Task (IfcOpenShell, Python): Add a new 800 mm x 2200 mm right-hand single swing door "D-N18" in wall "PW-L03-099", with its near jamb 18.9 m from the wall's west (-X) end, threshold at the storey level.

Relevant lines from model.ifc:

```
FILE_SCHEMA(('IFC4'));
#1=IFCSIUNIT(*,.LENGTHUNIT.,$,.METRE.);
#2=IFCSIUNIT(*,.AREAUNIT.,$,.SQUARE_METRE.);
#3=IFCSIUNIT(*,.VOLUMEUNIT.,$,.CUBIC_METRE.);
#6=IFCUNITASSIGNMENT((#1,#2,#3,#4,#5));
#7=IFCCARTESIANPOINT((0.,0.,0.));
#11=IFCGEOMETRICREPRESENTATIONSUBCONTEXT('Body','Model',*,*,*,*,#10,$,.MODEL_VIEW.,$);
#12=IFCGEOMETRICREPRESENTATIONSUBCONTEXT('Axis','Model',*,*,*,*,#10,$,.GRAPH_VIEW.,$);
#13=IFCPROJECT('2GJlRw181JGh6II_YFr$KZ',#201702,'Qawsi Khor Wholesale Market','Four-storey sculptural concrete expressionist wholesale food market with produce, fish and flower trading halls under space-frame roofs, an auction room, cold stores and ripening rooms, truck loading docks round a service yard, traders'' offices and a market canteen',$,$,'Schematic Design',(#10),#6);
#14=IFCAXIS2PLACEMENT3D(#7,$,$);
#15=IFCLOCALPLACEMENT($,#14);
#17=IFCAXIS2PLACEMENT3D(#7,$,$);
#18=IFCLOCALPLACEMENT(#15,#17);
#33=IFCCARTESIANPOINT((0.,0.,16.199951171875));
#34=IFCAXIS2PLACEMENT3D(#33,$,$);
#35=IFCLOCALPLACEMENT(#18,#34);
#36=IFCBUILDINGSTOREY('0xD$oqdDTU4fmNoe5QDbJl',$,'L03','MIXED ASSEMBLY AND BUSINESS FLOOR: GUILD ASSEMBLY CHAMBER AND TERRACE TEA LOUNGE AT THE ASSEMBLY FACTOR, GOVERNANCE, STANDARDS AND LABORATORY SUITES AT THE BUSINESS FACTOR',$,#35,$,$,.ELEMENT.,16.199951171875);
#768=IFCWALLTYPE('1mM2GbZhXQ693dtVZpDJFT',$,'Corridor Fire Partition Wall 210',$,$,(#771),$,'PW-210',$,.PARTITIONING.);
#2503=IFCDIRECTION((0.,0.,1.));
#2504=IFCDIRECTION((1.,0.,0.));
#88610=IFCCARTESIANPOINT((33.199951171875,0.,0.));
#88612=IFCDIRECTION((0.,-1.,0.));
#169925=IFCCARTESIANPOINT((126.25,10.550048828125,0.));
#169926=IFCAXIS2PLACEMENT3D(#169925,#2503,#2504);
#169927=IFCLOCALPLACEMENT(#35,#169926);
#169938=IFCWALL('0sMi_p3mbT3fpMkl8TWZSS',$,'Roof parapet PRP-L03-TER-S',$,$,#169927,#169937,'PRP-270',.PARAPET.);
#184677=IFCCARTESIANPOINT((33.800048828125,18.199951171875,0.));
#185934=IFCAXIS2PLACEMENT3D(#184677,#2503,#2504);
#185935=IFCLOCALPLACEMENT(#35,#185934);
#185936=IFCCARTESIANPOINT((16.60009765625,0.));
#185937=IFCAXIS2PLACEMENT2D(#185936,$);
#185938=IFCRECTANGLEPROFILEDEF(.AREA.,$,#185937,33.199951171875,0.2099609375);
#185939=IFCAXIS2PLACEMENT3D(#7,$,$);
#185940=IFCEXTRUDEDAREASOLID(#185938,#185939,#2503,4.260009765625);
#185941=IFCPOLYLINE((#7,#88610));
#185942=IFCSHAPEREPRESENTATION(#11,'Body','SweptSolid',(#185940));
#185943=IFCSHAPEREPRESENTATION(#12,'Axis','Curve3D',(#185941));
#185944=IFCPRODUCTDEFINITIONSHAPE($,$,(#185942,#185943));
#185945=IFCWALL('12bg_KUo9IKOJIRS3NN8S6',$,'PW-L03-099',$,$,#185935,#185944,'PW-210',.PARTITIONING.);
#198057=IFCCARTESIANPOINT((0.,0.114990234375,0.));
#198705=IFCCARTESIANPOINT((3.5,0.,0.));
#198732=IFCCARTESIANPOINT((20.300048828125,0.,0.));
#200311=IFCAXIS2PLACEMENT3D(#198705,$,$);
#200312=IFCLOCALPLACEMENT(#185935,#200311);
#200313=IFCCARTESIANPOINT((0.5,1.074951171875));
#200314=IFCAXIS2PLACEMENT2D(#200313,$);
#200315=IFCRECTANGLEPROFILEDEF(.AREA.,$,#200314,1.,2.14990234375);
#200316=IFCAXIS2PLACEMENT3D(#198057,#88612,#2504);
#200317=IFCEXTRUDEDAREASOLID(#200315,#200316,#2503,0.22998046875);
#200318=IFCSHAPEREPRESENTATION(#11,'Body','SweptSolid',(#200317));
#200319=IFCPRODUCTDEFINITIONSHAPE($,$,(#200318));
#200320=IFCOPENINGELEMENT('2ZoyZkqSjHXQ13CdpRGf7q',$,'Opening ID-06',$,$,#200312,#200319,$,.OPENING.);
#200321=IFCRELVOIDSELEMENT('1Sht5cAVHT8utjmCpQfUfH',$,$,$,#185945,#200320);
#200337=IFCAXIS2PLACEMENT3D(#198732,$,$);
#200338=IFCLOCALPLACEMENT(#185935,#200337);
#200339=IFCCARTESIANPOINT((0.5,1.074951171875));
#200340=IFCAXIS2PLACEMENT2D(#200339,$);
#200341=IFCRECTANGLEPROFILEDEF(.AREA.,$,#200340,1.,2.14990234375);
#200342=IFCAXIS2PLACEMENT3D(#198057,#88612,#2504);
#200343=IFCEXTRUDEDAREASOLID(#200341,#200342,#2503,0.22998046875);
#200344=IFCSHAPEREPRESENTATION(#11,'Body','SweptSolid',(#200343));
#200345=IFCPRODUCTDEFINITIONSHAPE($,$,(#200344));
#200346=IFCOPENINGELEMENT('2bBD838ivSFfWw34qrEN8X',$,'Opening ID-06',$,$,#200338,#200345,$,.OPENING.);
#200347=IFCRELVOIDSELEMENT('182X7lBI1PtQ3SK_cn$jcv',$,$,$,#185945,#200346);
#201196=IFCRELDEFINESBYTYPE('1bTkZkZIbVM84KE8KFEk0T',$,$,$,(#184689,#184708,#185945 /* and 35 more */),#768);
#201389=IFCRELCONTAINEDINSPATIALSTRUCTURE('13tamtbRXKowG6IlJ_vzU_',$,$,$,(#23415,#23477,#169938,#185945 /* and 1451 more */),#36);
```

```python
import numpy as np
import ifcopenshell
import ifcopenshell.api.feature
import ifcopenshell.api.geometry
import ifcopenshell.api.root
import ifcopenshell.api.spatial
import ifcopenshell.geom
import ifcopenshell.util.element
import ifcopenshell.util.placement
import ifcopenshell.util.representation
import ifcopenshell.util.shape
import ifcopenshell.util.unit

model = ifcopenshell.open("model.ifc")
unit_scale = ifcopenshell.util.unit.calculate_unit_scale(model)
settings = ifcopenshell.geom.settings()


def volume(element):
    """Net volume in cubic metres, openings subtracted."""
    shape = ifcopenshell.geom.create_shape(settings, element)
    return ifcopenshell.util.shape.get_volume(shape.geometry)


wall = model.by_guid("12bg_KUo9IKOJIRS3NN8S6")
storey = ifcopenshell.util.element.get_container(wall, ifc_class="IfcBuildingStorey")
context = ifcopenshell.util.representation.get_context(model, "Model", "Body", "MODEL_VIEW")
before = volume(wall)

width, height, from_end, sill = 0.8, 2.2, 18.9, 0.0  # metres

# The wall runs along its own X axis, and the end named is its -X end.
wall_shape = ifcopenshell.geom.create_shape(settings, wall)
x, y, z = ifcopenshell.util.shape.get_vertices(wall_shape.geometry).T
start = x.min() + from_end
face, thickness = float(y.min()), float(y.max() - y.min())
wall_matrix = ifcopenshell.util.placement.get_local_placement(wall.ObjectPlacement)
level = ifcopenshell.util.placement.get_local_placement(storey.ObjectPlacement)[2, 3]


def in_wall(x, y):
    """Placement at x, y metres in the wall's axes, at sill height."""
    matrix = wall_matrix.copy()
    matrix[:, 3] = wall_matrix @ np.array([x / unit_scale, y / unit_scale, 0.0, 1.0])
    matrix[2, 3] = level + sill / unit_scale
    return matrix


# Opening: a box that overshoots both wall faces by 50 mm.
opening = ifcopenshell.api.root.create_entity(model, ifc_class="IfcOpeningElement", predefined_type="OPENING")
box = ifcopenshell.api.geometry.add_wall_representation(
    model, context=context, length=width, height=height, thickness=thickness + 0.1
)
ifcopenshell.api.geometry.assign_representation(model, product=opening, representation=box)
ifcopenshell.api.geometry.edit_object_placement(model, product=opening, matrix=in_wall(start, face - 0.05), is_si=False)
ifcopenshell.api.feature.add_feature(model, feature=opening, element=wall)

door = ifcopenshell.api.root.create_entity(model, ifc_class="IfcDoor", name="D-N18", predefined_type="DOOR")
door.OverallWidth, door.OverallHeight = width / unit_scale, height / unit_scale
door.OperationType = "SINGLE_SWING_RIGHT"
body = ifcopenshell.api.geometry.add_door_representation(
    model,
    context=context,
    overall_width=door.OverallWidth,
    overall_height=door.OverallHeight,
    operation_type="SINGLE_SWING_RIGHT",
    lining_properties={"LiningDepth": thickness / unit_scale, "ThresholdDepth": thickness / unit_scale},
)
ifcopenshell.api.geometry.assign_representation(model, product=door, representation=body)
ifcopenshell.api.spatial.assign_container(model, products=[door], relating_structure=storey)
ifcopenshell.api.feature.add_filling(model, opening=opening, element=door)

# The lining spans the wall, so the door starts at the wall face.
ifcopenshell.api.geometry.edit_object_placement(model, product=door, matrix=in_wall(start, face), is_si=False)

after = volume(wall)

print(f"wall volume {before:.3f} -> {after:.3f} m3")

model.write("model_rev.ifc")
```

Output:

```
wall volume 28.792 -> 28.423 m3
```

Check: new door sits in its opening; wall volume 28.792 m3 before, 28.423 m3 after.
